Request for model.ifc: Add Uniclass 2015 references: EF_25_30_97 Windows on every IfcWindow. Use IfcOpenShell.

First a look at what the model holds.

```python
import ifcopenshell

model = ifcopenshell.open("model.ifc")
print(model.schema)
print("classifications:", [c.Name for c in model.by_type("IfcClassification")])
for ifc_class in ("IfcDoor", "IfcRoof", "IfcStair", "IfcWall", "IfcWindow"):
    print(ifc_class, len(model.by_type(ifc_class)))
```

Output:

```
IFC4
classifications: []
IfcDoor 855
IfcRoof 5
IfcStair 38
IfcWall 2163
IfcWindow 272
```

```python
import ifcopenshell
import ifcopenshell.api.classification

model = ifcopenshell.open("model.ifc")

system = ifcopenshell.api.classification.add_classification(model, classification="Uniclass 2015")

codes = {
    "IfcWindow": ("EF_25_30_97", "Windows"),
}
for ifc_class, (code, name) in codes.items():
    products = model.by_type(ifc_class)
    ifcopenshell.api.classification.add_reference(
        model, products=products, classification=system, identification=code, name=name
    )
    print(code, len(products))

model.write("model_edited.ifc")
```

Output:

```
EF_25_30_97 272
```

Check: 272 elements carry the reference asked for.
